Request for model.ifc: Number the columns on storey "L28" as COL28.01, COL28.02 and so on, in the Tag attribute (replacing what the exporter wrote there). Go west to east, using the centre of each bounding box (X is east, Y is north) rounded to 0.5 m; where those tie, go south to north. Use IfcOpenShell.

First a look at what the model holds.

```python
import ifcopenshell
import ifcopenshell.util.element
import ifcopenshell.util.placement

model = ifcopenshell.open("model.ifc")
print(model.schema)
storey = next(s for s in model.by_type("IfcBuildingStorey") if s.Name == "L28")
columns = [e for e in ifcopenshell.util.element.get_decomposition(storey) if e.is_a("IfcColumn")]
for e in sorted(columns, key=lambda e: e.id()):
    origin = ifcopenshell.util.placement.get_local_placement(e.ObjectPlacement)[:3, 3]
    print(e.id(), e.Tag, e.Name, origin.round(2) + 0.0, sep=" | ")
```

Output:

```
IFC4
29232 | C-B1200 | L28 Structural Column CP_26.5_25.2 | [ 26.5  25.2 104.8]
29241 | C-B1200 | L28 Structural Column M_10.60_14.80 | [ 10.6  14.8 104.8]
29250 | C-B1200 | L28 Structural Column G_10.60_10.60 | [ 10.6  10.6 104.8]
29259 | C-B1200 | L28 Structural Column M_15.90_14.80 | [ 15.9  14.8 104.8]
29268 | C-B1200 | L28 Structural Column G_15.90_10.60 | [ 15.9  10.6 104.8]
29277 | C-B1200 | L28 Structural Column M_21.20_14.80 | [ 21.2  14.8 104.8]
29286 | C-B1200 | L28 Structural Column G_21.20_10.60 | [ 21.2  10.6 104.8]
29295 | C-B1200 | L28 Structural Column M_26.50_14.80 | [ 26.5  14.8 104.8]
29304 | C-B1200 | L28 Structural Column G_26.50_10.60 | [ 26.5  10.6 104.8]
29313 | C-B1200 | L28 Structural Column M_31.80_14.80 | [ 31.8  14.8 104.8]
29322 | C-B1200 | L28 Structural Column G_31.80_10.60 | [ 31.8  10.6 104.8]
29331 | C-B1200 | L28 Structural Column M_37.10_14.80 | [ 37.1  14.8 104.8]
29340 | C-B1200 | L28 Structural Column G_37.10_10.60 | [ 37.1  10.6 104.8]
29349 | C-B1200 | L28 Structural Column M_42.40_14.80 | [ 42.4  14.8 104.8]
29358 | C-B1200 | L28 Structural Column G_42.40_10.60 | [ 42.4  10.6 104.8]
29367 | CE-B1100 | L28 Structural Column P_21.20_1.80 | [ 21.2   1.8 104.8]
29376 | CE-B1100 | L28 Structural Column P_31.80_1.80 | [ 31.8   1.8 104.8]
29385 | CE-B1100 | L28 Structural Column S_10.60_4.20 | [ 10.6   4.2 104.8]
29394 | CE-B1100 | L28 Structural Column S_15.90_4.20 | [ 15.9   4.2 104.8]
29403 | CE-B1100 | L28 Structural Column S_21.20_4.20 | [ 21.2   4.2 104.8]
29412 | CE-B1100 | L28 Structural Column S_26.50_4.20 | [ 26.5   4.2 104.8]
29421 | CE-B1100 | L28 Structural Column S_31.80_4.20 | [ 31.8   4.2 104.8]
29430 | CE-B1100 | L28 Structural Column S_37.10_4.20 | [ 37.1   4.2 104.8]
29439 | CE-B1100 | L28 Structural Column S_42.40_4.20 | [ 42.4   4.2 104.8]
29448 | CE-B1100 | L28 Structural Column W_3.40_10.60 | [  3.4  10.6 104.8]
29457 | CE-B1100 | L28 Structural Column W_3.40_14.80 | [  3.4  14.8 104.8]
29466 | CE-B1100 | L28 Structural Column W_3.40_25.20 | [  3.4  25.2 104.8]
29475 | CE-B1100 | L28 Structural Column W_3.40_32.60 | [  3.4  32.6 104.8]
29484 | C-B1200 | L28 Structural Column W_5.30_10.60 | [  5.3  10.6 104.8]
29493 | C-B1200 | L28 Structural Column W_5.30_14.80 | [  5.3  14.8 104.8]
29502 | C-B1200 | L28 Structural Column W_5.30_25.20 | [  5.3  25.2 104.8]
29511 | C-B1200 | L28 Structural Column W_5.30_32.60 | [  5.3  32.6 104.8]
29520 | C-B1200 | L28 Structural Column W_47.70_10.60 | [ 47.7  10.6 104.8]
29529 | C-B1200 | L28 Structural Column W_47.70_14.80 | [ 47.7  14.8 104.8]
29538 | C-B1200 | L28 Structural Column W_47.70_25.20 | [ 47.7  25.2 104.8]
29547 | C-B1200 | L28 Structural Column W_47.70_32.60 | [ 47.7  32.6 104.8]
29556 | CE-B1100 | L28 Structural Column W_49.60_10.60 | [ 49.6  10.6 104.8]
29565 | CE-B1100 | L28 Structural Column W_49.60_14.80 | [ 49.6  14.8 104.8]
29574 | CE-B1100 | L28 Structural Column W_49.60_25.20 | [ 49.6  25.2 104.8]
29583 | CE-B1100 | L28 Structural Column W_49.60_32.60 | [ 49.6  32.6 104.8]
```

```python
import ifcopenshell
import ifcopenshell.geom
import ifcopenshell.util.element
import ifcopenshell.util.shape

model = ifcopenshell.open("model.ifc")
settings = ifcopenshell.geom.settings()
settings.set("use-world-coords", True)


def centre(element):
    shape = ifcopenshell.geom.create_shape(settings, element)
    return ifcopenshell.util.shape.get_bbox_centroid(shape.geometry)


storey = next(s for s in model.by_type("IfcBuildingStorey") if s.Name == "L28")
columns = [e for e in ifcopenshell.util.element.get_decomposition(storey) if e.is_a("IfcColumn")]

# Insertion points can sit at a corner or the storey origin, so sort by the geometry (in metres).
centres = {e: centre(e) for e in columns}
columns.sort(key=lambda e: (round(centres[e][0] / 0.5), centres[e][1]))

for i, e in enumerate(columns, start=1):
    number = f"COL28.{i:02d}"
    e.Tag = number
    print(e.id(), number)

model.write("model_rev.ifc")
```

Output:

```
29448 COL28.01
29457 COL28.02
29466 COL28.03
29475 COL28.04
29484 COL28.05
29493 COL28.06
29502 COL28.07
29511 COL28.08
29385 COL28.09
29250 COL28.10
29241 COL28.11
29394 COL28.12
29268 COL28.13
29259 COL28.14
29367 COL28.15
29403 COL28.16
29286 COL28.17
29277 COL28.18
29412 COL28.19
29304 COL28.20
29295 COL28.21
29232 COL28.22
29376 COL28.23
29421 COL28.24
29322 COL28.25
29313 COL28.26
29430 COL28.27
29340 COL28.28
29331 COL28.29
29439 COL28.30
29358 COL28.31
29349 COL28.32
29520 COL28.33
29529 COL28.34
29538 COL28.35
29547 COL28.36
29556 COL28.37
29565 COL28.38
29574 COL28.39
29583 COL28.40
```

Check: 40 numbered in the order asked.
